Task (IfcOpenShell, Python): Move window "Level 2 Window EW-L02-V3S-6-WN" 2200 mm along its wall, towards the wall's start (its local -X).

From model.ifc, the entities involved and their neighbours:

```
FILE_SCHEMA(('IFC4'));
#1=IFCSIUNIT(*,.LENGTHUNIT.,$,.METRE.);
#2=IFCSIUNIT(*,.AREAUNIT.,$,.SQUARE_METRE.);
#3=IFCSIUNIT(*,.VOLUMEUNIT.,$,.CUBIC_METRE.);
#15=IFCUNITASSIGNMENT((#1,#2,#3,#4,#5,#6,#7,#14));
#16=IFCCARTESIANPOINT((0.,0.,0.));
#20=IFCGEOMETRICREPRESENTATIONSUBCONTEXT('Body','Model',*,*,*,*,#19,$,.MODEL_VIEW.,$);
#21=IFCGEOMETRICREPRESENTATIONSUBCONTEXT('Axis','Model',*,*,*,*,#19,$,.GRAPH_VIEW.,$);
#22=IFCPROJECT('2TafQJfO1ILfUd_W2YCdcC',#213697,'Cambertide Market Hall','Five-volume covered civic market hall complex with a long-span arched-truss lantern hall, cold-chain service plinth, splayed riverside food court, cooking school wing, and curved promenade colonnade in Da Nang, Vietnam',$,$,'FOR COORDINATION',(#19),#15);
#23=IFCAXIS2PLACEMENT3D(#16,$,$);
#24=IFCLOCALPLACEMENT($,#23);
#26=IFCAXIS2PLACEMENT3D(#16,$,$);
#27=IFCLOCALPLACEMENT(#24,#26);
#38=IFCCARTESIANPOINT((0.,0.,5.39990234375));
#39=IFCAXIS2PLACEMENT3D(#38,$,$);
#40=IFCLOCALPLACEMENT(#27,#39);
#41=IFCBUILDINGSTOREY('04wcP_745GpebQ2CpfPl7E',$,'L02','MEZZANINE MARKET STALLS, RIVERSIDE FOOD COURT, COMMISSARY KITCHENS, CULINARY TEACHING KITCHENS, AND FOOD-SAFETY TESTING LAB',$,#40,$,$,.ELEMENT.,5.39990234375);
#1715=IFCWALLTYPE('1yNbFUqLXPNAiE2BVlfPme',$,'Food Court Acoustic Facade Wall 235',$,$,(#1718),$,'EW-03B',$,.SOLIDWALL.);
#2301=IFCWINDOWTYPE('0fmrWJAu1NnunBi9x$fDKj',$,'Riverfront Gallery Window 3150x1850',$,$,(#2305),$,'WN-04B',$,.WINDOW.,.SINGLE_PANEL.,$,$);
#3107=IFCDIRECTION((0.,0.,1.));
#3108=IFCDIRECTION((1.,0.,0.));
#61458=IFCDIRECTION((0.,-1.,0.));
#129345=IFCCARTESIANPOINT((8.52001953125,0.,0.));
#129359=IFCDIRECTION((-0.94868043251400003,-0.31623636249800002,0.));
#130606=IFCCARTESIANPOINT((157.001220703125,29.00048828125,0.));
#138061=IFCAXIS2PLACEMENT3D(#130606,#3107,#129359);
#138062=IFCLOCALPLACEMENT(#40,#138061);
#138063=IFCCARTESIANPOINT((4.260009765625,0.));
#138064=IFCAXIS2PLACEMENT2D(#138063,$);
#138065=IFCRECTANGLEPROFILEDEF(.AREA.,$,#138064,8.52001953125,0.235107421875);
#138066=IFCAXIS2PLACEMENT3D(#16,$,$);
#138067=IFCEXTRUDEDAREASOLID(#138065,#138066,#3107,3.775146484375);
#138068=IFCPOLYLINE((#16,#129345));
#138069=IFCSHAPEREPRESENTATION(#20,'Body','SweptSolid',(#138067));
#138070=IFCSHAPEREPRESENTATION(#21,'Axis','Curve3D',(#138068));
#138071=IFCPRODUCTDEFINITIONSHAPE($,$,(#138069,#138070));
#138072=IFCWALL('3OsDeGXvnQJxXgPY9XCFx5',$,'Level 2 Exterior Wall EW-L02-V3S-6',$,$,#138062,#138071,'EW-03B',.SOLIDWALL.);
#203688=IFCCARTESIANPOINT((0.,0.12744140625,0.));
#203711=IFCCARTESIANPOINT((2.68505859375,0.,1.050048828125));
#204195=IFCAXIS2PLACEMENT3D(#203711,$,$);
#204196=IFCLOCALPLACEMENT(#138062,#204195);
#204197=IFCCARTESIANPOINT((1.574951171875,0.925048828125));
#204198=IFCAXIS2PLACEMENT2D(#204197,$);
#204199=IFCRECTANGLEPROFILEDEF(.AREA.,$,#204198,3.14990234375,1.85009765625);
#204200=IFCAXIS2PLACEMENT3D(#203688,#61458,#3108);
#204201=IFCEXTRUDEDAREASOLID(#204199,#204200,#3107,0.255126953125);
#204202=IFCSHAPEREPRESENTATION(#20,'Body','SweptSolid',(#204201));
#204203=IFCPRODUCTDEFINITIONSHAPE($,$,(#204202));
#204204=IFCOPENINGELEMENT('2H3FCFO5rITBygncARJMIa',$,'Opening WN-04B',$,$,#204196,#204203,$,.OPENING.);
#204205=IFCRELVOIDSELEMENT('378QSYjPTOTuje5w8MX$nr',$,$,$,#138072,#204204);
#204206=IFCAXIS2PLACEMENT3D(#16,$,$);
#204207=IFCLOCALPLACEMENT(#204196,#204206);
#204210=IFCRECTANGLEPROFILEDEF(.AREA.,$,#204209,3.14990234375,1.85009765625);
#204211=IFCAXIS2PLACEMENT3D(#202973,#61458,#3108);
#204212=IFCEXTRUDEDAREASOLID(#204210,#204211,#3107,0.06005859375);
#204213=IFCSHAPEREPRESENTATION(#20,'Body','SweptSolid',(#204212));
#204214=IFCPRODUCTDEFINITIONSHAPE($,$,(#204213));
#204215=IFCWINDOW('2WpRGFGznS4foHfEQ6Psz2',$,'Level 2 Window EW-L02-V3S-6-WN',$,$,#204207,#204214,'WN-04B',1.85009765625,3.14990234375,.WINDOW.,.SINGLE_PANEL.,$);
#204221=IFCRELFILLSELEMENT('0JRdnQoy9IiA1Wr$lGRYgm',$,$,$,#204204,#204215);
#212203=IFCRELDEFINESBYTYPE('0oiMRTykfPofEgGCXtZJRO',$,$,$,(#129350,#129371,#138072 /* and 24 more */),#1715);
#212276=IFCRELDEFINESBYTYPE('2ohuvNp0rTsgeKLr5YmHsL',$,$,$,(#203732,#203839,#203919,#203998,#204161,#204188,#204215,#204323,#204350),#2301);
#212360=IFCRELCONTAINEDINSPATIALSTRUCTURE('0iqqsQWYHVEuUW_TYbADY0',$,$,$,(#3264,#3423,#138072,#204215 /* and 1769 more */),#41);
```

```python
import ifcopenshell
import ifcopenshell.api.geometry
import ifcopenshell.util.placement

model = ifcopenshell.open("model.ifc")

window = model.by_guid("2WpRGFGznS4foHfEQ6Psz2")
opening = window.FillsVoids[0].RelatingOpeningElement
wall = opening.VoidsElements[0].RelatingBuildingElement

wall_matrix = ifcopenshell.util.placement.get_local_placement(wall.ObjectPlacement)
shift = wall_matrix[:3, 0] * -2.2
before = ifcopenshell.util.placement.get_local_placement(window.ObjectPlacement)[:3, 3].copy()

# The window is placed relative to its opening, so it follows when the opening moves.
matrix = ifcopenshell.util.placement.get_local_placement(opening.ObjectPlacement)
matrix[:3, 3] += shift
ifcopenshell.api.geometry.edit_object_placement(
    model, product=opening, matrix=matrix, is_si=False, should_transform_children=True
)

after = ifcopenshell.util.placement.get_local_placement(window.ObjectPlacement)[:3, 3]
print("window moved by", (after - before).round(3) + 0.0)

model.write("model-out.ifc")
```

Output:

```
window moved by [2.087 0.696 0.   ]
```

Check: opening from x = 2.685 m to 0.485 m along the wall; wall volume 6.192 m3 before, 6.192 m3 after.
